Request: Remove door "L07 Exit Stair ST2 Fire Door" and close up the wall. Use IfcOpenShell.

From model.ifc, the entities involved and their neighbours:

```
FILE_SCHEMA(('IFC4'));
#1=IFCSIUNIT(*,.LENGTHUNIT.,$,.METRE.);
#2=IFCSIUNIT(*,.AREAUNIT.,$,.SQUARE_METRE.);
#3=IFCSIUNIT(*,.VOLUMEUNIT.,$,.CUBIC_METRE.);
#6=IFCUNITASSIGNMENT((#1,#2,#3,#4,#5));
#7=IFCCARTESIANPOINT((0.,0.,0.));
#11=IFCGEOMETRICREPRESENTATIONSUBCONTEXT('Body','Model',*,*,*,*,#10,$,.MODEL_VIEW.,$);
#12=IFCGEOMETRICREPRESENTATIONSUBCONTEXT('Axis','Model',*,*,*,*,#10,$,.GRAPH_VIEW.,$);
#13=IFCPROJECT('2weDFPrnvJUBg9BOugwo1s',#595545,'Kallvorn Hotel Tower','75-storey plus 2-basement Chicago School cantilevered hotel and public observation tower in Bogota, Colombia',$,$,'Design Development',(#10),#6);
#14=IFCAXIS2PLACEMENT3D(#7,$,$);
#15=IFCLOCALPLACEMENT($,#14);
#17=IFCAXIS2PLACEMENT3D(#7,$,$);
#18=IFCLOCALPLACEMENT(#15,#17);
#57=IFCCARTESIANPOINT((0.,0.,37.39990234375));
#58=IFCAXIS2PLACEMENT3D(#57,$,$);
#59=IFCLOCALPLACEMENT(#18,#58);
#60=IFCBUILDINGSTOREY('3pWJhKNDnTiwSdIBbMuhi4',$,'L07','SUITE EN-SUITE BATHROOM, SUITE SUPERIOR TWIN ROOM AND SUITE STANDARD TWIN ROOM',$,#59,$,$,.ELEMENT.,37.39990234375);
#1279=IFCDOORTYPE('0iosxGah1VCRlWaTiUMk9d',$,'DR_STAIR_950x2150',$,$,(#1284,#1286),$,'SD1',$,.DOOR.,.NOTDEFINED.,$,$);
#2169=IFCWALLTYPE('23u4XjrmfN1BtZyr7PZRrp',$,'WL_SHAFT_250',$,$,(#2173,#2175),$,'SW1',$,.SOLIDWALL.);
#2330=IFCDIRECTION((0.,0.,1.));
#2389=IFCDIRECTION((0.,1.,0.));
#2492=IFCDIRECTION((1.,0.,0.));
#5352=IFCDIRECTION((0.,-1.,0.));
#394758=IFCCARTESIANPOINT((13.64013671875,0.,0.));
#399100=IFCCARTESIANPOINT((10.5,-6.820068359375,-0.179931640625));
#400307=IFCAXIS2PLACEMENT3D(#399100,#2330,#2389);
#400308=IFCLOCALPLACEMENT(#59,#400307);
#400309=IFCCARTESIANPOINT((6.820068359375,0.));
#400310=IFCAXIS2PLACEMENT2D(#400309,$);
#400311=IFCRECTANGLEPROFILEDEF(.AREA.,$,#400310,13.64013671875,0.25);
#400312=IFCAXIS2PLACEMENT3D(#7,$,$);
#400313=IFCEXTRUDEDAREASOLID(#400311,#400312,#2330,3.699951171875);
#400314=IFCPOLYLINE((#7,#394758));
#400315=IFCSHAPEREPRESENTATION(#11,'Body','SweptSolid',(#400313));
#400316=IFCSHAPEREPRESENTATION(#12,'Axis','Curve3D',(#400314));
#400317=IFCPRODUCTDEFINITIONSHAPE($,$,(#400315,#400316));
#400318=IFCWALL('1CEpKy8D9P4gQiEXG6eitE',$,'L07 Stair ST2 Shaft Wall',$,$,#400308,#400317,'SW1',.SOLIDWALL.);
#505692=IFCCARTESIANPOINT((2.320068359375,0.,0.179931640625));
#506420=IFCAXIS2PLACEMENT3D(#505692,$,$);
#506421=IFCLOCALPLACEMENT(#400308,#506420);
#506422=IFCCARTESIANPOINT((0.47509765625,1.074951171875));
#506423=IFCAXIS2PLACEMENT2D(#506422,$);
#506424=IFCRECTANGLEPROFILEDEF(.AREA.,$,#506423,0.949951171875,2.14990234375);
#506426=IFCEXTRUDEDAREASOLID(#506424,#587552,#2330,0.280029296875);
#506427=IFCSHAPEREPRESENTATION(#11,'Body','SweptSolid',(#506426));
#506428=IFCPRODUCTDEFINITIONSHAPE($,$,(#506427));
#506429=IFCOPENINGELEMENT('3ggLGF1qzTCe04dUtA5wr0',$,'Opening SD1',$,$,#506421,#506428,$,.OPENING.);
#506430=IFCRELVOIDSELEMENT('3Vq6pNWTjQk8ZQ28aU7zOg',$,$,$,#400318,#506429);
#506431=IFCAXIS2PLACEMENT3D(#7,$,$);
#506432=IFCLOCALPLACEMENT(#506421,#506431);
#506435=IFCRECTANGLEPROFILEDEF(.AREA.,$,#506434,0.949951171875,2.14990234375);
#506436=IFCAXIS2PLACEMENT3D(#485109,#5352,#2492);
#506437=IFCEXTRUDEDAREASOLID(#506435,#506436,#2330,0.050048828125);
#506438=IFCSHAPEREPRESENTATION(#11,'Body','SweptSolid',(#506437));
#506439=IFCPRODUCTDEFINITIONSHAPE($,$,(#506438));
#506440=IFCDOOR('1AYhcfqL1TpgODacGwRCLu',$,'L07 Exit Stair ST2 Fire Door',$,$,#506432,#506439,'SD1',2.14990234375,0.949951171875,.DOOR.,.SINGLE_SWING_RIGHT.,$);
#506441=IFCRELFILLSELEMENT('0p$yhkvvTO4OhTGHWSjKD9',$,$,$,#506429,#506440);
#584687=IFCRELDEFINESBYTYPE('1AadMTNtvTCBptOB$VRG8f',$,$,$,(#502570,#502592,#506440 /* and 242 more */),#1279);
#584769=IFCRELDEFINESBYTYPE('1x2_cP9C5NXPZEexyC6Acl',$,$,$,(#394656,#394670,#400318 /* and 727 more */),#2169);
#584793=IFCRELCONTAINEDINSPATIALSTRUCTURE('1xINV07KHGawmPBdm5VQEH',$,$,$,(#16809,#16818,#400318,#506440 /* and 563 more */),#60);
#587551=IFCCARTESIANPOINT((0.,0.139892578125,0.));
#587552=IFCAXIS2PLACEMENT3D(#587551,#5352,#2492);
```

```python
import ifcopenshell
import ifcopenshell.api.feature
import ifcopenshell.api.root
import ifcopenshell.geom
import ifcopenshell.util.shape

model = ifcopenshell.open("model.ifc")
settings = ifcopenshell.geom.settings()


def volume(element):
    """Net volume in cubic metres, openings subtracted."""
    shape = ifcopenshell.geom.create_shape(settings, element)
    return ifcopenshell.util.shape.get_volume(shape.geometry)


door = model.by_guid("1AYhcfqL1TpgODacGwRCLu")
opening = door.FillsVoids[0].RelatingOpeningElement
wall = opening.VoidsElements[0].RelatingBuildingElement
before = volume(wall)

ifcopenshell.api.root.remove_product(model, product=door)
ifcopenshell.api.feature.remove_feature(model, feature=opening)

after = volume(wall)

print(f"wall volume {before:.3f} -> {after:.3f} m3")

model.write("model_rev.ifc")
```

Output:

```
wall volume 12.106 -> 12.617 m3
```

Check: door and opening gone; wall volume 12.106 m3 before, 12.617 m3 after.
